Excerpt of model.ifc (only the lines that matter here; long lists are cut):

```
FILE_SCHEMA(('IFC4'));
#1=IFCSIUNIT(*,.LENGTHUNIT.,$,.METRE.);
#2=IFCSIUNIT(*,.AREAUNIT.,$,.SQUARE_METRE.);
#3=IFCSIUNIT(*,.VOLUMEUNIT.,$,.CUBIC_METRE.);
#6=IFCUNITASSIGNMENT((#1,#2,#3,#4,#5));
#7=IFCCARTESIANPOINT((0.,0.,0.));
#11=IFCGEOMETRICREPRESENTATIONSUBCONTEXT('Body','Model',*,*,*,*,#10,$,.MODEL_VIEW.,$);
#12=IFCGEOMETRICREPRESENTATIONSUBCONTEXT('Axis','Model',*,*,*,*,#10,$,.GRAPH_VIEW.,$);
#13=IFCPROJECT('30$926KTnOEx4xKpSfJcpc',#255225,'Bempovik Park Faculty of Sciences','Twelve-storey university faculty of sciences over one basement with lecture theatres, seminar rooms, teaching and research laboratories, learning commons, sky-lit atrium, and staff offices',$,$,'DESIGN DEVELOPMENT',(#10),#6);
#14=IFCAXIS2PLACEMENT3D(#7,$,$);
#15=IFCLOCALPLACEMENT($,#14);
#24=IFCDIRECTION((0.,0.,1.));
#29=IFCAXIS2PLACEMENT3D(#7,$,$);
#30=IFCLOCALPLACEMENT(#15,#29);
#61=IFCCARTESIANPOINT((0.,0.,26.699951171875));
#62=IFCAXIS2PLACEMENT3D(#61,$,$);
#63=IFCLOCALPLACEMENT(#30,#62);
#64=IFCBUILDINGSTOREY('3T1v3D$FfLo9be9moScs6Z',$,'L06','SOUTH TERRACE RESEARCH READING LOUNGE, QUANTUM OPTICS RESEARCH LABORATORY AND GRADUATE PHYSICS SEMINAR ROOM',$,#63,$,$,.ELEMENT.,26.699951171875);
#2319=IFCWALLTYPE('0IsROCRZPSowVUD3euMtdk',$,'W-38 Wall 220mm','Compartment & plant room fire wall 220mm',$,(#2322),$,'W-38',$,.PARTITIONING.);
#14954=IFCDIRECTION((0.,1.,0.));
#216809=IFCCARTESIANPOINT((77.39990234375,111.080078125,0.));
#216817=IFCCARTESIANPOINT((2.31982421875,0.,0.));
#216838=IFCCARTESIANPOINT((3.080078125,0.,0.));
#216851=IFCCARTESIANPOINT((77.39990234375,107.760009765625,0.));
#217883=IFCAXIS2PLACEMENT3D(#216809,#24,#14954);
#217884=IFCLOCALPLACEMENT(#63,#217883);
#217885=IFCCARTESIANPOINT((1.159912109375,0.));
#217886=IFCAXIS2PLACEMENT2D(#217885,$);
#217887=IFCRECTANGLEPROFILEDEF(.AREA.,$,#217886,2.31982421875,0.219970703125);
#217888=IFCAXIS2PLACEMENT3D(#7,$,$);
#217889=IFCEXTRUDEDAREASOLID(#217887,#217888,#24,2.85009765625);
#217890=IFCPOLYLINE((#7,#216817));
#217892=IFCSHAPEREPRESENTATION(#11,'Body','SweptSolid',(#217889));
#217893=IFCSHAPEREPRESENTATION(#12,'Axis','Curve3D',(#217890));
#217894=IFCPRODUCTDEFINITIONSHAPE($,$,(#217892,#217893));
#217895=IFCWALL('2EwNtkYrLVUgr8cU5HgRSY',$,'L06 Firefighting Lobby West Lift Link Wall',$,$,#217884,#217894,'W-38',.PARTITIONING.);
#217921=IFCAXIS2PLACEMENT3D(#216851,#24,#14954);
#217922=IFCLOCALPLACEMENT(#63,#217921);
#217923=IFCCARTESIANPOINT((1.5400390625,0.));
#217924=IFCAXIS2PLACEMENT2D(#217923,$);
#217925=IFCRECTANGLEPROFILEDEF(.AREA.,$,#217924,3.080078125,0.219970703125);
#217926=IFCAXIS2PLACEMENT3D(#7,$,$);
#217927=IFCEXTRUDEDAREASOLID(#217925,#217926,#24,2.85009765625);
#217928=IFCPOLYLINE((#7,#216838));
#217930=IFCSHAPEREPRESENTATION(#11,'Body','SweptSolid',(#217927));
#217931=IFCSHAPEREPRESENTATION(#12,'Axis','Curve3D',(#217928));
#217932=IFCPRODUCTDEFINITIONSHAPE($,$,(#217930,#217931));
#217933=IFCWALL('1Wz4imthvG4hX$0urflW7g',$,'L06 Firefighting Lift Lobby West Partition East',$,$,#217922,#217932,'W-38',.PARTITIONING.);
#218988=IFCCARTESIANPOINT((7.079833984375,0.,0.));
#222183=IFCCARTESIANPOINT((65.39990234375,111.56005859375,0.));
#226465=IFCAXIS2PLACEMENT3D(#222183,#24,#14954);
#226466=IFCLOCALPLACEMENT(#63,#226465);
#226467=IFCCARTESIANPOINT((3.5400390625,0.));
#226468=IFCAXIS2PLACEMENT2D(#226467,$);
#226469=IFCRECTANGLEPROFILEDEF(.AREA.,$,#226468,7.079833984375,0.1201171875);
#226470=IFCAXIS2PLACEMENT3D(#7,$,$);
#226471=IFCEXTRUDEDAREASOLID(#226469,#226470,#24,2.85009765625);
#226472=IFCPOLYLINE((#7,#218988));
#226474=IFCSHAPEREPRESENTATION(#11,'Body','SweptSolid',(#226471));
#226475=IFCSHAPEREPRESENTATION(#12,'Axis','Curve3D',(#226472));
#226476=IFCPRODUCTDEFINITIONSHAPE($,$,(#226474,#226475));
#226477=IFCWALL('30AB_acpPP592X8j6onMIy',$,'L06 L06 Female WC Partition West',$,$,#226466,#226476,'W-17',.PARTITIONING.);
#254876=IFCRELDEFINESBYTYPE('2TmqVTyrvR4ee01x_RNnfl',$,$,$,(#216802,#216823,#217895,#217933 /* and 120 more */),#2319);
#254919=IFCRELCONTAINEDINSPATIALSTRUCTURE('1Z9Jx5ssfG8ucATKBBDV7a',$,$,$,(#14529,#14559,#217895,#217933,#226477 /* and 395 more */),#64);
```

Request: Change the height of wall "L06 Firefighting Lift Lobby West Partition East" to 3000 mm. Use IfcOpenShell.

```python
import ifcopenshell
import ifcopenshell.geom
import ifcopenshell.util.representation
import ifcopenshell.util.shape

model = ifcopenshell.open("model.ifc")
settings = ifcopenshell.geom.settings()


def volume(element):
    """Net volume in cubic metres, openings subtracted."""
    shape = ifcopenshell.geom.create_shape(settings, element)
    return ifcopenshell.util.shape.get_volume(shape.geometry)


wall = model.by_id(217933)
before = volume(wall)

body = ifcopenshell.util.representation.get_representation(wall, "Model", "Body")
solid = body.Items[0]
old_height = solid.Depth
solid.Depth = 3.0
after = volume(wall)

print(f"height {old_height:g} -> {solid.Depth:g}, volume {before:.3f} -> {after:.3f} m3")

model.write("model-out.ifc")
```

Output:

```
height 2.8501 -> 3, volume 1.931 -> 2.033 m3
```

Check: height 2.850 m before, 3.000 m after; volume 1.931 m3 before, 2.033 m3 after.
